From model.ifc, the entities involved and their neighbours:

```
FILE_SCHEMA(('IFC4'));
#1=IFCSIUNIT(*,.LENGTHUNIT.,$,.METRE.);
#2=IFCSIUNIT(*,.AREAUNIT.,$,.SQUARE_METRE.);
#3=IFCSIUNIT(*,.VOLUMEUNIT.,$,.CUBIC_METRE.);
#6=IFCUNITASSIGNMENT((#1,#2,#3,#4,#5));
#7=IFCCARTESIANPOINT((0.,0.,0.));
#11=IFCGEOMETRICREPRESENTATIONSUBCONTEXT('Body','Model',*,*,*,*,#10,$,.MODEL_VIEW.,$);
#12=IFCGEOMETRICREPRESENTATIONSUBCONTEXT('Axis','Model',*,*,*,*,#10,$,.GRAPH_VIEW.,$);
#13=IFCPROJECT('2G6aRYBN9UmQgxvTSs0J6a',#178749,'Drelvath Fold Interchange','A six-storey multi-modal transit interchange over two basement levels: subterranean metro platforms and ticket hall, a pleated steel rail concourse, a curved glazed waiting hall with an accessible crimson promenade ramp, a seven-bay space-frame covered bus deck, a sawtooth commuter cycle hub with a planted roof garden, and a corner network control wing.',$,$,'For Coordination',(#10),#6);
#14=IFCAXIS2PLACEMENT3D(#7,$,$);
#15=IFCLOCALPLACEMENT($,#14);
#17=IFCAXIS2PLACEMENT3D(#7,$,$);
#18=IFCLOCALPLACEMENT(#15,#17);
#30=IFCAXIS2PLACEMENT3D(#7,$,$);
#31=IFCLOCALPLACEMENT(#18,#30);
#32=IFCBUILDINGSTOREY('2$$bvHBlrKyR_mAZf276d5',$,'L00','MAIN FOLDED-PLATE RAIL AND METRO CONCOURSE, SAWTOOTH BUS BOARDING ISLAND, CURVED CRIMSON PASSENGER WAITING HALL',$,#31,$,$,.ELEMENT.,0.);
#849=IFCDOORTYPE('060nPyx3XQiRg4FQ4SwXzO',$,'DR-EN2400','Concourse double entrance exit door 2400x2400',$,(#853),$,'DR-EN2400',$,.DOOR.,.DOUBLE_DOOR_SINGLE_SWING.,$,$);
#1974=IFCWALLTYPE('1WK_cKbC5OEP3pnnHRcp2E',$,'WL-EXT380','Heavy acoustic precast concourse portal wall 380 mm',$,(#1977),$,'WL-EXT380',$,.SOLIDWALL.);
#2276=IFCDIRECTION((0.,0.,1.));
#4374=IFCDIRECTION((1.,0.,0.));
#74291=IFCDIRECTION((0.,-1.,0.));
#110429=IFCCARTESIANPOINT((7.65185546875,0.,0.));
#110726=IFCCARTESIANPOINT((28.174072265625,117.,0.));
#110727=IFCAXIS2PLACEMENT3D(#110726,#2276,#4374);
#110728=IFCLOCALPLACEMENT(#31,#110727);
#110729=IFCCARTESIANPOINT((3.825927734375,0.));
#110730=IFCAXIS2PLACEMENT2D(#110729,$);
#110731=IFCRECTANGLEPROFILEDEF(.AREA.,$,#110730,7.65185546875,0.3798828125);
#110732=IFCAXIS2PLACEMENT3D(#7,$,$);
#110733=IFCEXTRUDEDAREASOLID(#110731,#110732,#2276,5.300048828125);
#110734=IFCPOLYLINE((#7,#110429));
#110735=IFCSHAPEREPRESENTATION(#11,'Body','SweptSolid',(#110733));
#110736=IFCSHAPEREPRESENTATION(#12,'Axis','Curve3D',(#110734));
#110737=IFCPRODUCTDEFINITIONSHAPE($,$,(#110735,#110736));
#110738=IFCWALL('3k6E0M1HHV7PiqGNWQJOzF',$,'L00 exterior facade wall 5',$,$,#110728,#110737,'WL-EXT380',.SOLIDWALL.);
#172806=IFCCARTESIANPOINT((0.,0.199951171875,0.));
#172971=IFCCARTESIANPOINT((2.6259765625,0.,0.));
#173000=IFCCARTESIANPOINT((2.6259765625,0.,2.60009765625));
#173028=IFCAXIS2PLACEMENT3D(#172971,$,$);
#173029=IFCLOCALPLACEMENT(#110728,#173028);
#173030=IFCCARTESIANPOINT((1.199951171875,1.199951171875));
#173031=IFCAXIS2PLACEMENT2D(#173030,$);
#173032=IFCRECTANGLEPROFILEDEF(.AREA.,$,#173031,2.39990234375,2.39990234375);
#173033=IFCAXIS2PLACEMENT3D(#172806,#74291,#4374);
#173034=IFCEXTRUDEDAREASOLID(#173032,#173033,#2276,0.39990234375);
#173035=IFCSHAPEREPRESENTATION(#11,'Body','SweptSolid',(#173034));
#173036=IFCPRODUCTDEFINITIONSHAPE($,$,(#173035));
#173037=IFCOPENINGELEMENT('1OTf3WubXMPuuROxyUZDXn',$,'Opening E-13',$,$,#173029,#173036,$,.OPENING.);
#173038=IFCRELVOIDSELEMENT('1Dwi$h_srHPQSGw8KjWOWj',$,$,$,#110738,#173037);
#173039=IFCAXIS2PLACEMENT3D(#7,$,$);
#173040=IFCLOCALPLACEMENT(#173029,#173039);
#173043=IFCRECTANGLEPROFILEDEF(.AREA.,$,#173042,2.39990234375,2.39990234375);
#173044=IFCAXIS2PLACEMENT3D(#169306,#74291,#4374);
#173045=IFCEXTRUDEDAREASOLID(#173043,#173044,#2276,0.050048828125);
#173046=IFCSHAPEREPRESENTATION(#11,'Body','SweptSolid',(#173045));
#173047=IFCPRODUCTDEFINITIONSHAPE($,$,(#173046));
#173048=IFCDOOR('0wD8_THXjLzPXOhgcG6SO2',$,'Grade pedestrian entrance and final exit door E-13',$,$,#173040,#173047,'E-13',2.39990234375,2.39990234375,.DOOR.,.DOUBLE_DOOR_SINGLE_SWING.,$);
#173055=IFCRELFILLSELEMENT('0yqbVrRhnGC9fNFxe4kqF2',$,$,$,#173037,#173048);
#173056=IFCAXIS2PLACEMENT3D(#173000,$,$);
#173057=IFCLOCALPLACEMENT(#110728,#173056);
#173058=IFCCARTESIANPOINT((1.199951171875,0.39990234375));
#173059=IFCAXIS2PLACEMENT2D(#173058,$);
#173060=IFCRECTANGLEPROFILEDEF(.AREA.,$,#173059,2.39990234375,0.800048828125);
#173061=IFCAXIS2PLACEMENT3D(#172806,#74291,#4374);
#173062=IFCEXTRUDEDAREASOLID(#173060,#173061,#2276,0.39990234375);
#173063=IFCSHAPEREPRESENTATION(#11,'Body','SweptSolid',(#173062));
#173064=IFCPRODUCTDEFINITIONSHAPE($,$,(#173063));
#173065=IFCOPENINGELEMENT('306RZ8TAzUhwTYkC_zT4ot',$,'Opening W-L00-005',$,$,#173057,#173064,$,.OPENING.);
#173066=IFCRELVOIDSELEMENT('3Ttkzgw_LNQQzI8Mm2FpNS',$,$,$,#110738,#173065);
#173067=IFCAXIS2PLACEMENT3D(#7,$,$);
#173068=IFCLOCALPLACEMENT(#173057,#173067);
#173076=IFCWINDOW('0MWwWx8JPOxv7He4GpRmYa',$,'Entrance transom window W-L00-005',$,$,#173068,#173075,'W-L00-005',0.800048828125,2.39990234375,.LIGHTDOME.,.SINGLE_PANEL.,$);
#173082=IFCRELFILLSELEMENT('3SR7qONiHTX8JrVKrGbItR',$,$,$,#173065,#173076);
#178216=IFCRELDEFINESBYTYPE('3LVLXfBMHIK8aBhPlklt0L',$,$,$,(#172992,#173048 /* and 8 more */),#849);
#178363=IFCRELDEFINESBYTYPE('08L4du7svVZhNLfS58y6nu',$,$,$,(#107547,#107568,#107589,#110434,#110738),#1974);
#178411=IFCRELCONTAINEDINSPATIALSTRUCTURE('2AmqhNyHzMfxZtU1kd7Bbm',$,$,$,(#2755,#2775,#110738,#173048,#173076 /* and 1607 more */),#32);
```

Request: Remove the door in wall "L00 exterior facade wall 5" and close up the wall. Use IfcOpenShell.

```python
import ifcopenshell
import ifcopenshell.api.feature
import ifcopenshell.api.root
import ifcopenshell.geom
import ifcopenshell.util.shape

model = ifcopenshell.open("model.ifc")
settings = ifcopenshell.geom.settings()


def volume(element):
    """Net volume in cubic metres, openings subtracted."""
    shape = ifcopenshell.geom.create_shape(settings, element)
    return ifcopenshell.util.shape.get_volume(shape.geometry)


door = model.by_guid("0wD8_THXjLzPXOhgcG6SO2")
opening = door.FillsVoids[0].RelatingOpeningElement
wall = opening.VoidsElements[0].RelatingBuildingElement
before = volume(wall)

ifcopenshell.api.root.remove_product(model, product=door)
ifcopenshell.api.feature.remove_feature(model, feature=opening)

after = volume(wall)

print(f"wall volume {before:.3f} -> {after:.3f} m3")

model.write("model_rev.ifc")
```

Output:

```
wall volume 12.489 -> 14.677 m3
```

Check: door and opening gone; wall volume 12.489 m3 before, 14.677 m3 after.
